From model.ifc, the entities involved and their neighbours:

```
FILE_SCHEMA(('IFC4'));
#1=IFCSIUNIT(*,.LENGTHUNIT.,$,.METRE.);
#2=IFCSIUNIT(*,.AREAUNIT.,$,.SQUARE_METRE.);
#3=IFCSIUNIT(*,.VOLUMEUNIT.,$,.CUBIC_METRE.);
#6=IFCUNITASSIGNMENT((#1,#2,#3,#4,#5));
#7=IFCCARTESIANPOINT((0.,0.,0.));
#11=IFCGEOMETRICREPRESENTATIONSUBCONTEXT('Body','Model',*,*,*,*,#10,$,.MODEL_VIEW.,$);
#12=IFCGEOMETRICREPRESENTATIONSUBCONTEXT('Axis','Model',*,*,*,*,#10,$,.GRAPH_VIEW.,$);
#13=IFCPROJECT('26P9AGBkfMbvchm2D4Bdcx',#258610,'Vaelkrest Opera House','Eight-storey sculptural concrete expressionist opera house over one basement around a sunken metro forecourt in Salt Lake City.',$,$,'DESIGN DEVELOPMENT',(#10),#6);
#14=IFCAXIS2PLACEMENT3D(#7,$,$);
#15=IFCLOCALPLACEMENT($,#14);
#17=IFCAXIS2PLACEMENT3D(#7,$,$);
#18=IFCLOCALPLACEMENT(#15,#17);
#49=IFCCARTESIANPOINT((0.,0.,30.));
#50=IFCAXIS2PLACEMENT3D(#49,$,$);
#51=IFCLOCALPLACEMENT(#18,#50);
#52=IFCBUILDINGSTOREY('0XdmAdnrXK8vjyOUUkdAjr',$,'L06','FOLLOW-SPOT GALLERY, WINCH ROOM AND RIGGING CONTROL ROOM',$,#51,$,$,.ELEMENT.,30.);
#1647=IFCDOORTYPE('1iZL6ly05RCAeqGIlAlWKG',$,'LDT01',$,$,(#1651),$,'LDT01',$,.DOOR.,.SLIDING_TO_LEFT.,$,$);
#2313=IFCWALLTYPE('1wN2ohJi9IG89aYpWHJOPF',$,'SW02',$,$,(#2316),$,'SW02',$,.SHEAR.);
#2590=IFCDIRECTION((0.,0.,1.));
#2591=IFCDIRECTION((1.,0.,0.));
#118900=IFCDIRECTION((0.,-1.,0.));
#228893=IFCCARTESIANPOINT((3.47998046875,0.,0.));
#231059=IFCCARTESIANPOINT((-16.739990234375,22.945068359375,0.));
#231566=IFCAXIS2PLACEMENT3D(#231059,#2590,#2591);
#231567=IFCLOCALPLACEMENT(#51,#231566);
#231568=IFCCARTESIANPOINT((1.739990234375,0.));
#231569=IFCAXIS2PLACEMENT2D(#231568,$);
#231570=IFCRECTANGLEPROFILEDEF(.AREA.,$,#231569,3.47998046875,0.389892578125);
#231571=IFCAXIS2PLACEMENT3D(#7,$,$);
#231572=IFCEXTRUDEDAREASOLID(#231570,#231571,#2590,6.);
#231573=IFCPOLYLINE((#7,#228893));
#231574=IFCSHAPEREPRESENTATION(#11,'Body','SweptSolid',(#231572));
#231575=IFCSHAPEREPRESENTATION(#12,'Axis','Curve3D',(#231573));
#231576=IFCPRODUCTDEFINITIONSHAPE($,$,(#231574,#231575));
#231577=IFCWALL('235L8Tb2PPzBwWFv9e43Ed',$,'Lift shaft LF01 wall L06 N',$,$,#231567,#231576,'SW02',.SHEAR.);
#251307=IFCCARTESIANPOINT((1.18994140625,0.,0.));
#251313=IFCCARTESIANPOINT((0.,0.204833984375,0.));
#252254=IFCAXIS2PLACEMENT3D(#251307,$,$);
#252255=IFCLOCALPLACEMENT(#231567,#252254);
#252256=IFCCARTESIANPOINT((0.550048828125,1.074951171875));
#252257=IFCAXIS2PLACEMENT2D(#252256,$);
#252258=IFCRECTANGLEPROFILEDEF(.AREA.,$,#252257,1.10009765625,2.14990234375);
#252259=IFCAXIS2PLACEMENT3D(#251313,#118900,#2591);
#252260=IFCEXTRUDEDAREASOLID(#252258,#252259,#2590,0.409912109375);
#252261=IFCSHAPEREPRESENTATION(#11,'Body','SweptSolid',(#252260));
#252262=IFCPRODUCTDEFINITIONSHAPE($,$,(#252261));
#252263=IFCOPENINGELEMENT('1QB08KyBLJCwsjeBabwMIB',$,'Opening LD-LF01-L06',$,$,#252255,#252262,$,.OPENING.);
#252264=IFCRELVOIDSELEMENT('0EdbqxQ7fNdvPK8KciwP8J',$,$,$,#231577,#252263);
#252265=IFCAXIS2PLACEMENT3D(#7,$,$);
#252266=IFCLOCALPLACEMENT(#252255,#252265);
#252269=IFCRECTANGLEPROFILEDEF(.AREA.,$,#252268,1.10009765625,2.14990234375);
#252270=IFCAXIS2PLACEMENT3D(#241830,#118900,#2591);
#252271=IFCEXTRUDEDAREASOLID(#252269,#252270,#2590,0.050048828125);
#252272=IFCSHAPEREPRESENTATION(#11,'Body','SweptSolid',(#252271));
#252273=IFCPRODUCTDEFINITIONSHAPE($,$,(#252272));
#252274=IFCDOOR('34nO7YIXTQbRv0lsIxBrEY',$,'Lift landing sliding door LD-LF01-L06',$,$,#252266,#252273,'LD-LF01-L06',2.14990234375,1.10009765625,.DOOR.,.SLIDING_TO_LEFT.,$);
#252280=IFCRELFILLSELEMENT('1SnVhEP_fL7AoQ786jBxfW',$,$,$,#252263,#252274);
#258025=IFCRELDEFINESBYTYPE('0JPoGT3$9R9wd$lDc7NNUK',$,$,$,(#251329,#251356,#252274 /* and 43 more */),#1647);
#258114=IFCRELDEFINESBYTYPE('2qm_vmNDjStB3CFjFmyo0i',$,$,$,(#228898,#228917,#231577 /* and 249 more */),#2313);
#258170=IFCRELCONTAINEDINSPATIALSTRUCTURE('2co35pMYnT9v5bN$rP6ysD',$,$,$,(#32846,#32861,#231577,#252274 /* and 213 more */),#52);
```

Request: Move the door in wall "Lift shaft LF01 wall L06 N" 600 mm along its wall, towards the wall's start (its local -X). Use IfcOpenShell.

```python
import ifcopenshell
import ifcopenshell.api.geometry
import ifcopenshell.util.placement
import ifcopenshell.util.unit

model = ifcopenshell.open("model.ifc")
unit_scale = ifcopenshell.util.unit.calculate_unit_scale(model)

door = model.by_guid("34nO7YIXTQbRv0lsIxBrEY")
opening = door.FillsVoids[0].RelatingOpeningElement
wall = opening.VoidsElements[0].RelatingBuildingElement

wall_matrix = ifcopenshell.util.placement.get_local_placement(wall.ObjectPlacement)
shift = wall_matrix[:3, 0] * -0.6 / unit_scale
before = ifcopenshell.util.placement.get_local_placement(door.ObjectPlacement)[:3, 3].copy()

# The door is placed relative to its opening, so it follows when the opening moves.
matrix = ifcopenshell.util.placement.get_local_placement(opening.ObjectPlacement)
matrix[:3, 3] += shift
ifcopenshell.api.geometry.edit_object_placement(
    model, product=opening, matrix=matrix, is_si=False, should_transform_children=True
)

after = ifcopenshell.util.placement.get_local_placement(door.ObjectPlacement)[:3, 3]
print("door moved by", (after - before).round(3) + 0.0)

model.write("model-out.ifc")
```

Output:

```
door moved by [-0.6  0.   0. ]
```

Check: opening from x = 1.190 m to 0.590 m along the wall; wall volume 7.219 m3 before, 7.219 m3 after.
